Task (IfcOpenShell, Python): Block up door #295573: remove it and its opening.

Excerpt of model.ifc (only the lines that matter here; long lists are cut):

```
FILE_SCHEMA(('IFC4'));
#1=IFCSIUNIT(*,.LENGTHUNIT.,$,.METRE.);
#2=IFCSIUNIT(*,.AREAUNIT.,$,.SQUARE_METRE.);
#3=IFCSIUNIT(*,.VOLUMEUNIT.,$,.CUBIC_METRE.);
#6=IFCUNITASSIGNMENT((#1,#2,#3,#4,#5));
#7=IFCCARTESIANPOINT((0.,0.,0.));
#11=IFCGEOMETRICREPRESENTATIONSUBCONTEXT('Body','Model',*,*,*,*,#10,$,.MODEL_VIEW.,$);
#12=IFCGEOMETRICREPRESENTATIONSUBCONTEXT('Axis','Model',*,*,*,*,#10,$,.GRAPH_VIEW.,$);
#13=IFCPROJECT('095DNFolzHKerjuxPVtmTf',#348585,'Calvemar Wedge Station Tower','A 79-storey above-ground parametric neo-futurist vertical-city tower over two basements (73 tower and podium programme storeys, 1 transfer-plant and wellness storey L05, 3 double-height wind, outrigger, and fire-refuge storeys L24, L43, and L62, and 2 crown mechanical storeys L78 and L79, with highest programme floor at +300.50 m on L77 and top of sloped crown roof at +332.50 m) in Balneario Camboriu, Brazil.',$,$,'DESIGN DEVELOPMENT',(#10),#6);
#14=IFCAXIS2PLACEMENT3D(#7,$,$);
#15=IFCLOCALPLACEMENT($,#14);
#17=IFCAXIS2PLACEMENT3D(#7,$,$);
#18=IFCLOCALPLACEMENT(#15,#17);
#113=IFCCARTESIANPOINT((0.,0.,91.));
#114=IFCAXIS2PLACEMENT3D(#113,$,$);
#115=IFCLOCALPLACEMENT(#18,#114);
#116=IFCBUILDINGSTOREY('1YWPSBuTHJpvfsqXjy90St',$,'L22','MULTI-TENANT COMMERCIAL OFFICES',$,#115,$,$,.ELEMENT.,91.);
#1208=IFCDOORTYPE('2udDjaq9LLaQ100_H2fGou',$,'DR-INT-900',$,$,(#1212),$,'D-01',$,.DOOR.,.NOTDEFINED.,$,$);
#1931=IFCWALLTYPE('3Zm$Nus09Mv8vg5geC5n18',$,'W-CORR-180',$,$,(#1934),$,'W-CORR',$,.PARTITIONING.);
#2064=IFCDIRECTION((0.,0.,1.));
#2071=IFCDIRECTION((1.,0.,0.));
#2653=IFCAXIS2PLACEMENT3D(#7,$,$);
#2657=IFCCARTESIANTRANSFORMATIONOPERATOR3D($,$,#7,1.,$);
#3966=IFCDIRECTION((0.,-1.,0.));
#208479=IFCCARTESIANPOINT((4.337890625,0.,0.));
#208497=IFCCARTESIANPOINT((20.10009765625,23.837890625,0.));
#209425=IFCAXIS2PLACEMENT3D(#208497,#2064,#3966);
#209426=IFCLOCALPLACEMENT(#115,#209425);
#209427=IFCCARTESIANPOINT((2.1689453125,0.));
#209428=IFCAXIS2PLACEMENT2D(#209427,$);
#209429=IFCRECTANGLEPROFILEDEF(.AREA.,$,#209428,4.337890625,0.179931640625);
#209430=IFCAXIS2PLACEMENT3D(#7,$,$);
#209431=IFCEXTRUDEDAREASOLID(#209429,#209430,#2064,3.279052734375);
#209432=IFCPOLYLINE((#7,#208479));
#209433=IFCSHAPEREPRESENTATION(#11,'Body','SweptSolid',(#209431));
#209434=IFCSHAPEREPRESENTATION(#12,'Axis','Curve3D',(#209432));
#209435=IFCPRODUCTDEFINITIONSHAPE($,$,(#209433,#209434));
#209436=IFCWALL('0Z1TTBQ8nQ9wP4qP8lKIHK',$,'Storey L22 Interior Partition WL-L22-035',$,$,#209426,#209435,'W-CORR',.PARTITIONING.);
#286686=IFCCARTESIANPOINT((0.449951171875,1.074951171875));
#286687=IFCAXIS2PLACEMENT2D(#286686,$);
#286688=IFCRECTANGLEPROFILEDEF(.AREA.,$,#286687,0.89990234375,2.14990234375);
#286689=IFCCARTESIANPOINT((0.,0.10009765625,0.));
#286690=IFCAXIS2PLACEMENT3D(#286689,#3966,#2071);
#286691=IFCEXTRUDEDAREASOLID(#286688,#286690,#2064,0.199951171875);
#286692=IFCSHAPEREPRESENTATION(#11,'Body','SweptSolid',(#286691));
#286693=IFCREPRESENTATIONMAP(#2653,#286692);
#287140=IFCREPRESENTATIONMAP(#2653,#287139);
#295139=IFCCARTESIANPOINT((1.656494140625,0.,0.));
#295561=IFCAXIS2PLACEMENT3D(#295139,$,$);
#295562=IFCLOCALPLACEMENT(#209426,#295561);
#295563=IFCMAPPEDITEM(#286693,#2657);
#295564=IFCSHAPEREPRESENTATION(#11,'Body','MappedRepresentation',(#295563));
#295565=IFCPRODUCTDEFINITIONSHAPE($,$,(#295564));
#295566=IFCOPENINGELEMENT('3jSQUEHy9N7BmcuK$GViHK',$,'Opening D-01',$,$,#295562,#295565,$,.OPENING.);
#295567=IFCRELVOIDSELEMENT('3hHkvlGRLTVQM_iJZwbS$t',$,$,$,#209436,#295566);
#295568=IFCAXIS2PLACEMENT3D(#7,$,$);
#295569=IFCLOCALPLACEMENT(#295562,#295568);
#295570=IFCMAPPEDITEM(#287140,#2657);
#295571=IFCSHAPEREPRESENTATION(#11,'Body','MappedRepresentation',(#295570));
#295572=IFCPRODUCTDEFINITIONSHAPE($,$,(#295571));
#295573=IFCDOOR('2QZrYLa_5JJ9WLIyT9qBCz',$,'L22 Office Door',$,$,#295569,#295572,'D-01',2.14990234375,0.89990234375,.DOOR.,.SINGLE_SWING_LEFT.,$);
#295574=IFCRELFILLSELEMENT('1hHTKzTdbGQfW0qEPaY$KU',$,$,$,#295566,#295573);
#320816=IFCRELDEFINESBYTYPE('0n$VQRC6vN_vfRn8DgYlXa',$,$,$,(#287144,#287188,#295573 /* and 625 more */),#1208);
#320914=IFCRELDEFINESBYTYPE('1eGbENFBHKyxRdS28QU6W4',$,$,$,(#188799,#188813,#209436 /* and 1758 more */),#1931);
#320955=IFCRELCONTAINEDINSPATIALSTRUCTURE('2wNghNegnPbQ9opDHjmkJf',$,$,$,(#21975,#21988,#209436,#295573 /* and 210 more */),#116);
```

```python
import ifcopenshell
import ifcopenshell.api.feature
import ifcopenshell.api.root
import ifcopenshell.geom
import ifcopenshell.util.shape

model = ifcopenshell.open("model.ifc")
settings = ifcopenshell.geom.settings()


def volume(element):
    """Net volume in cubic metres, openings subtracted."""
    shape = ifcopenshell.geom.create_shape(settings, element)
    return ifcopenshell.util.shape.get_volume(shape.geometry)


door = model.by_guid("2QZrYLa_5JJ9WLIyT9qBCz")
opening = door.FillsVoids[0].RelatingOpeningElement
wall = opening.VoidsElements[0].RelatingBuildingElement
before = volume(wall)

ifcopenshell.api.root.remove_product(model, product=door)
ifcopenshell.api.feature.remove_feature(model, feature=opening)

after = volume(wall)

print(f"wall volume {before:.3f} -> {after:.3f} m3")

model.write("model_rev.ifc")
```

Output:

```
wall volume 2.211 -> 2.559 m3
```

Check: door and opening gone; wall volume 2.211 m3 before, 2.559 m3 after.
